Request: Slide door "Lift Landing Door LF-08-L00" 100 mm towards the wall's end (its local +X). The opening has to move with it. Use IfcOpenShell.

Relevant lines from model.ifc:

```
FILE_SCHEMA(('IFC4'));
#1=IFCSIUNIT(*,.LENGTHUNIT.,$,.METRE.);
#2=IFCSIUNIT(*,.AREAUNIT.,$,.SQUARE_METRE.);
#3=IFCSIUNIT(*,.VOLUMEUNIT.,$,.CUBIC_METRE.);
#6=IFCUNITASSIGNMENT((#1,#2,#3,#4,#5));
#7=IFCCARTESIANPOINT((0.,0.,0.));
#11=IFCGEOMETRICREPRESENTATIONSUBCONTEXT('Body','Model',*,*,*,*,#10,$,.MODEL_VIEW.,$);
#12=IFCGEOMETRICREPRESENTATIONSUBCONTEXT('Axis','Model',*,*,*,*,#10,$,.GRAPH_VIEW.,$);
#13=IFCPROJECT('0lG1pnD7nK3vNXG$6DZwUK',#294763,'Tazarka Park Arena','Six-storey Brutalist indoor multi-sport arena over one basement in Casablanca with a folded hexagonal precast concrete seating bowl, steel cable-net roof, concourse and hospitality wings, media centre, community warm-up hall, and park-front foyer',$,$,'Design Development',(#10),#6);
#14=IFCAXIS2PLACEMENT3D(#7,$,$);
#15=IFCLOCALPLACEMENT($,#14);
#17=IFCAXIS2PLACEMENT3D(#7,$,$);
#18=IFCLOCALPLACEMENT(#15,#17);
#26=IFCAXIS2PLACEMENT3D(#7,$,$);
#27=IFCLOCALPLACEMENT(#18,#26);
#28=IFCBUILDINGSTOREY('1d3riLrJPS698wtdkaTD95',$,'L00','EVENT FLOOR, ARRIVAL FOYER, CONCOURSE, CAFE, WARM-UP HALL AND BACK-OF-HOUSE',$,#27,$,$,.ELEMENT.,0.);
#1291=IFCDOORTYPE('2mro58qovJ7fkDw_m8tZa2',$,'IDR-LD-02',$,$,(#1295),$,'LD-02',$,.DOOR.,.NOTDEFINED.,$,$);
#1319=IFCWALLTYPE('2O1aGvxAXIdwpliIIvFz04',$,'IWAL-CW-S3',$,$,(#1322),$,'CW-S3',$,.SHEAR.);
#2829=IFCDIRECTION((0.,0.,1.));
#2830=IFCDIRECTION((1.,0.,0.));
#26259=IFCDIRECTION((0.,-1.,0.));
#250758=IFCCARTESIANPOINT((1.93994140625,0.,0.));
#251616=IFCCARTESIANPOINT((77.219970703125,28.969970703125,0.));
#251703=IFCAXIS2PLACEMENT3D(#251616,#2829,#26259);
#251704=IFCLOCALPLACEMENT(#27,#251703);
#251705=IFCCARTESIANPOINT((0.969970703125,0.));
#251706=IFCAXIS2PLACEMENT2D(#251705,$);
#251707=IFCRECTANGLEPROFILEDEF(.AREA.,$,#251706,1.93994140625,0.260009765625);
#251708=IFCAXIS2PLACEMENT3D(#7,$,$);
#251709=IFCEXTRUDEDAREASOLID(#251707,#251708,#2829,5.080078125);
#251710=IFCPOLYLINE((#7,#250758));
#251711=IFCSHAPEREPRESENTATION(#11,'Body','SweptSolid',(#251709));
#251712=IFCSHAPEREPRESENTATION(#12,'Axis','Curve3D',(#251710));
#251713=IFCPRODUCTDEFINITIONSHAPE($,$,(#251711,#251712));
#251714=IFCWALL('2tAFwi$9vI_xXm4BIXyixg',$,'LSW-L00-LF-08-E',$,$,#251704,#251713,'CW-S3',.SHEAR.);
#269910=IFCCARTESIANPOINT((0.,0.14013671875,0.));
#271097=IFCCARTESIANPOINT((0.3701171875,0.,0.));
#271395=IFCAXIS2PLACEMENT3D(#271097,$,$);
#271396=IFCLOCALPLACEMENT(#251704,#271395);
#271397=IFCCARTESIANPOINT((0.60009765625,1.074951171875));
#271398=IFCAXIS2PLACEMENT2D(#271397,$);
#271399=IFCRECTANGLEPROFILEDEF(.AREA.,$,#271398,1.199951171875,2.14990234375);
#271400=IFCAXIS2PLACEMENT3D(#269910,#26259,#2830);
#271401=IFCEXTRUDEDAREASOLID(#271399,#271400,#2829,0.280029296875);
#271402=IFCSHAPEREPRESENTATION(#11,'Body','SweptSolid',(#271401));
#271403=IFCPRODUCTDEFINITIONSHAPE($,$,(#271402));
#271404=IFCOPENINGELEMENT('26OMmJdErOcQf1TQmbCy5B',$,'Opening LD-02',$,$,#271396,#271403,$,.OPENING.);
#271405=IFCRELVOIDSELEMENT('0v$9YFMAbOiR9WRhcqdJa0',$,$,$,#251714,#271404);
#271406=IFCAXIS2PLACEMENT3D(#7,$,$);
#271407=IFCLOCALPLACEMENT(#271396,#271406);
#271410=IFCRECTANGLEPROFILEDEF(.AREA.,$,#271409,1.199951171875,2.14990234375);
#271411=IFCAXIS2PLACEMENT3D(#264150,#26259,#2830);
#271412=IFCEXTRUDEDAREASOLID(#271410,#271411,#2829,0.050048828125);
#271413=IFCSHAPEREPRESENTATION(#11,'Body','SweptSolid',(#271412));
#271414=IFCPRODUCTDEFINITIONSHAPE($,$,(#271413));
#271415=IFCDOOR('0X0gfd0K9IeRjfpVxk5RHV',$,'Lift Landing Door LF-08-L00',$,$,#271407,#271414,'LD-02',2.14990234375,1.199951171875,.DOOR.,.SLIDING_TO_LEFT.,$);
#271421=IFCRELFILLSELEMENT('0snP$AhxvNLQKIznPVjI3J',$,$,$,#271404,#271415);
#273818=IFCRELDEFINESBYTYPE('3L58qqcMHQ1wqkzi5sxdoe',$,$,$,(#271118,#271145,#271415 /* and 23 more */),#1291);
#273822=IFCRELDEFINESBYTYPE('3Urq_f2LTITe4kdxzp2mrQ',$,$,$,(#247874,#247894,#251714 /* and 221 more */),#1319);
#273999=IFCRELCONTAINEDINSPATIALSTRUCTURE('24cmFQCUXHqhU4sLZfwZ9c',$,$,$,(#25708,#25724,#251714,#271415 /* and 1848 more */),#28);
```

```python
import ifcopenshell
import ifcopenshell.api.geometry
import ifcopenshell.util.placement

model = ifcopenshell.open("model.ifc")

door = model.by_guid("0X0gfd0K9IeRjfpVxk5RHV")
opening = door.FillsVoids[0].RelatingOpeningElement
wall = opening.VoidsElements[0].RelatingBuildingElement

wall_matrix = ifcopenshell.util.placement.get_local_placement(wall.ObjectPlacement)
shift = wall_matrix[:3, 0] * 0.1
before = ifcopenshell.util.placement.get_local_placement(door.ObjectPlacement)[:3, 3].copy()

# The door is placed relative to its opening, so it follows when the opening moves.
matrix = ifcopenshell.util.placement.get_local_placement(opening.ObjectPlacement)
matrix[:3, 3] += shift
ifcopenshell.api.geometry.edit_object_placement(
    model, product=opening, matrix=matrix, is_si=False, should_transform_children=True
)

after = ifcopenshell.util.placement.get_local_placement(door.ObjectPlacement)[:3, 3]
print("door moved by", (after - before).round(3) + 0.0)

model.write("model_v2.ifc")
```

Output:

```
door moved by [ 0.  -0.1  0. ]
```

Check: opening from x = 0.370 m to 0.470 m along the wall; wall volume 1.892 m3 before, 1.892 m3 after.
